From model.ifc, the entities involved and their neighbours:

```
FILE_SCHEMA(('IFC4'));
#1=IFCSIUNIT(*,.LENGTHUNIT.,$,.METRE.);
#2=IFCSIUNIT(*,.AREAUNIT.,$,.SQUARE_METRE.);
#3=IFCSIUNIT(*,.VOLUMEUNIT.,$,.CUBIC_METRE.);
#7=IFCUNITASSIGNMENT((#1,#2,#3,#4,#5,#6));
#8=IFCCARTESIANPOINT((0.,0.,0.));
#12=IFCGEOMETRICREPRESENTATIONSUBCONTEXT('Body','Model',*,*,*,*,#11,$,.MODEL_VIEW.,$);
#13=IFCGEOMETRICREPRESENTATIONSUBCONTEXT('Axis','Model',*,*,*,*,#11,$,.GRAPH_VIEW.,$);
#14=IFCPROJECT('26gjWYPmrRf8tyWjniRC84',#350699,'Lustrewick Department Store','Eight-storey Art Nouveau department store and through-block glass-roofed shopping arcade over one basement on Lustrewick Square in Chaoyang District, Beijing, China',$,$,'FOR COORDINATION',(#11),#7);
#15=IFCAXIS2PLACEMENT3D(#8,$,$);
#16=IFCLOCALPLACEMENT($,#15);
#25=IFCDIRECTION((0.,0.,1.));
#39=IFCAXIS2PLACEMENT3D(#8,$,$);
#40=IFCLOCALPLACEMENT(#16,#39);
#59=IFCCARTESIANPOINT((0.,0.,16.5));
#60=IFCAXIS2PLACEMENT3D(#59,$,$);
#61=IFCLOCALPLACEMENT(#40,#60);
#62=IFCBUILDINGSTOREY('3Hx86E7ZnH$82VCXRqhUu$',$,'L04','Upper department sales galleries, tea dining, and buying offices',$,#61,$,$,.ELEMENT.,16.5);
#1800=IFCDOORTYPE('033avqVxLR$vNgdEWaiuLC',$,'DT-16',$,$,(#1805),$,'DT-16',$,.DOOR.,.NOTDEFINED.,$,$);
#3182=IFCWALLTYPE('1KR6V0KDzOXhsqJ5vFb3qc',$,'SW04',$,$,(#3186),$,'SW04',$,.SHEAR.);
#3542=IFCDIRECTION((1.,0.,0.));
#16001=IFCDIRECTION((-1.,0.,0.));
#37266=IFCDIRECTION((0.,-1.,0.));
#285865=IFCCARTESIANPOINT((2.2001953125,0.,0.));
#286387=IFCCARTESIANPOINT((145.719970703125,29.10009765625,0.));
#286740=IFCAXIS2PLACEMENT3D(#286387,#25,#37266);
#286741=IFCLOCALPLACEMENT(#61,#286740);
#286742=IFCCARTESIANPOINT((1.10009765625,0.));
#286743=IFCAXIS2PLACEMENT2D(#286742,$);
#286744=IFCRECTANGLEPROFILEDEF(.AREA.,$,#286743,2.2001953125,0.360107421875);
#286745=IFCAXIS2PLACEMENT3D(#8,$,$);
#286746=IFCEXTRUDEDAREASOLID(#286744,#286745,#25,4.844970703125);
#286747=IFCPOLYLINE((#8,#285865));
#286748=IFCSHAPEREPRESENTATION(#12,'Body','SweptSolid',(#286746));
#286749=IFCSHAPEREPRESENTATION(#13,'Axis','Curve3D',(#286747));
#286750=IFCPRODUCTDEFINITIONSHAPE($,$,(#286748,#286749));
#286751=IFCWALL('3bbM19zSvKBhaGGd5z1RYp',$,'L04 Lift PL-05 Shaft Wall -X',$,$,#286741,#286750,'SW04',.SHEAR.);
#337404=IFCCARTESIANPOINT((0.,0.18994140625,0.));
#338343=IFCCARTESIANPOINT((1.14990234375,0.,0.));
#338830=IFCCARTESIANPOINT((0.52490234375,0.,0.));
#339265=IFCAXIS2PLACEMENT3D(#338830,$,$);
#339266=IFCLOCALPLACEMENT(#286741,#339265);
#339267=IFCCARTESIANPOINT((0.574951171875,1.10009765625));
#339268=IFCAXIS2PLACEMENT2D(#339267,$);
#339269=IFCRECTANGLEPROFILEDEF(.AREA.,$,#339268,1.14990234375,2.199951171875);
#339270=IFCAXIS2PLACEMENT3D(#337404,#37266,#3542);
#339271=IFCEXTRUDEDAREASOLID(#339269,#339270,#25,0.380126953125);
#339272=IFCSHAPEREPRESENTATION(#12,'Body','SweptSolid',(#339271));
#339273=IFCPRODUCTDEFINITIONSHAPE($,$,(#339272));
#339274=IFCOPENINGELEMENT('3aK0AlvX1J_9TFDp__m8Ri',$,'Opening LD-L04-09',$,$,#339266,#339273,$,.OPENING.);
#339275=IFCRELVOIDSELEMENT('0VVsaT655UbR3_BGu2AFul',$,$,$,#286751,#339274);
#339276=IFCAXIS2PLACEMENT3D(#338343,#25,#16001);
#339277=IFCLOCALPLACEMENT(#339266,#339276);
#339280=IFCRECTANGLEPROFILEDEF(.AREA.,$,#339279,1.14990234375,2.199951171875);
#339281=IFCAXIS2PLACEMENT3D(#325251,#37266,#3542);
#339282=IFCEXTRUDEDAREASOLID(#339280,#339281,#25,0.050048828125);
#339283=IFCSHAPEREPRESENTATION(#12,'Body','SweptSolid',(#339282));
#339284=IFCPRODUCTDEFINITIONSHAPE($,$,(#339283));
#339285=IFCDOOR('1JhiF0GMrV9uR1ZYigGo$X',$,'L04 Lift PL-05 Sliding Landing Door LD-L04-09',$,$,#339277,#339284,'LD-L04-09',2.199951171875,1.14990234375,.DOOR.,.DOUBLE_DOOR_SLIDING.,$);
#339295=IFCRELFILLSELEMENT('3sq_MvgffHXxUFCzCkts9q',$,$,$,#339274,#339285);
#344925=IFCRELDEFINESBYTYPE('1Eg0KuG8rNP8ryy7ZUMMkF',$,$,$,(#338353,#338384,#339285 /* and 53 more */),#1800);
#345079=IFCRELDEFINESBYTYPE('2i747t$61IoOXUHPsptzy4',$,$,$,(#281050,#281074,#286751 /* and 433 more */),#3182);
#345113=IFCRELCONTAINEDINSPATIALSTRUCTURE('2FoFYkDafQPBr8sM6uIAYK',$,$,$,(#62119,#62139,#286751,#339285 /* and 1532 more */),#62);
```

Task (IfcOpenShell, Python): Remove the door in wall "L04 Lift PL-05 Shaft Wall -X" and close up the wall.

```python
import ifcopenshell
import ifcopenshell.api.feature
import ifcopenshell.api.root
import ifcopenshell.geom
import ifcopenshell.util.shape

model = ifcopenshell.open("model.ifc")
settings = ifcopenshell.geom.settings()


def volume(element):
    """Net volume in cubic metres, openings subtracted."""
    shape = ifcopenshell.geom.create_shape(settings, element)
    return ifcopenshell.util.shape.get_volume(shape.geometry)


door = model.by_id(339285)
opening = door.FillsVoids[0].RelatingOpeningElement
wall = opening.VoidsElements[0].RelatingBuildingElement
before = volume(wall)

ifcopenshell.api.root.remove_product(model, product=door)
ifcopenshell.api.feature.remove_feature(model, feature=opening)

after = volume(wall)

print(f"wall volume {before:.3f} -> {after:.3f} m3")

model.write("model_rev.ifc")
```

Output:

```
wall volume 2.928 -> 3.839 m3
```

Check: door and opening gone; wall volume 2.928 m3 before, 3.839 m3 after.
